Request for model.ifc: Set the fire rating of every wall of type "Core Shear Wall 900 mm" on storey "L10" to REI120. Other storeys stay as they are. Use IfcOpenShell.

First a look at what the model holds.

```python
import ifcopenshell
import ifcopenshell.util.element

model = ifcopenshell.open("model.ifc")
print(model.schema)
storey = next(s for s in model.by_type("IfcBuildingStorey") if s.Name == "L10")
walls = [e for e in ifcopenshell.util.element.get_decomposition(storey) if e.is_a("IfcWall")]
seen = {}
for e in walls:
    element_type = ifcopenshell.util.element.get_type(e)
    key = (element_type.Name if element_type != e and element_type else None, ifcopenshell.util.element.get_pset(e, "Pset_WallCommon", "FireRating"))
    seen[key] = seen.get(key, 0) + 1
for (name, value), count in sorted(seen.items(), key=str):
    print(count, "x", name, "|", value)
```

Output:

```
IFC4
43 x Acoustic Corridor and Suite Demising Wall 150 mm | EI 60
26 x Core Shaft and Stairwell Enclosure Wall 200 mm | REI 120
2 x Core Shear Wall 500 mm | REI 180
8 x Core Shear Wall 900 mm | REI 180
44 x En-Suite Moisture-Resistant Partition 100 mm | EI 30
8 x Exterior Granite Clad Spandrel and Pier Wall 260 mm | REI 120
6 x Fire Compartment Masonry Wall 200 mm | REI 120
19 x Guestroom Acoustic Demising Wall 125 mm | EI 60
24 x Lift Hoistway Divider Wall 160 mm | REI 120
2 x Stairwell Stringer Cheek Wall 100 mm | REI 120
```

```python
import ifcopenshell
import ifcopenshell.api.pset
import ifcopenshell.util.element

model = ifcopenshell.open("model.ifc")

storey = next(s for s in model.by_type("IfcBuildingStorey") if s.Name == "L10")
walls = [e for e in ifcopenshell.util.element.get_decomposition(storey) if e.is_a("IfcWall")]

count = 0
for e in walls:
    element_type = ifcopenshell.util.element.get_type(e)
    if element_type in (None, e) or element_type.Name != "Core Shear Wall 900 mm":
        continue
    found = ifcopenshell.util.element.get_pset(e, "Pset_WallCommon", should_inherit=False)
    if found:
        pset = model.by_id(found["id"])
        if len(ifcopenshell.util.element.get_elements_by_pset(pset)) > 1:
            pset = ifcopenshell.api.pset.unshare_pset(model, products=[e], pset=pset)[0]
    else:
        pset = ifcopenshell.api.pset.add_pset(model, product=e, name="Pset_WallCommon")
    ifcopenshell.api.pset.edit_pset(model, pset=pset, properties={"FireRating": "REI120"})
    count += 1

print(count, "walls updated")

model.write("model-out.ifc")
```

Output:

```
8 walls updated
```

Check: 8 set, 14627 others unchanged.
